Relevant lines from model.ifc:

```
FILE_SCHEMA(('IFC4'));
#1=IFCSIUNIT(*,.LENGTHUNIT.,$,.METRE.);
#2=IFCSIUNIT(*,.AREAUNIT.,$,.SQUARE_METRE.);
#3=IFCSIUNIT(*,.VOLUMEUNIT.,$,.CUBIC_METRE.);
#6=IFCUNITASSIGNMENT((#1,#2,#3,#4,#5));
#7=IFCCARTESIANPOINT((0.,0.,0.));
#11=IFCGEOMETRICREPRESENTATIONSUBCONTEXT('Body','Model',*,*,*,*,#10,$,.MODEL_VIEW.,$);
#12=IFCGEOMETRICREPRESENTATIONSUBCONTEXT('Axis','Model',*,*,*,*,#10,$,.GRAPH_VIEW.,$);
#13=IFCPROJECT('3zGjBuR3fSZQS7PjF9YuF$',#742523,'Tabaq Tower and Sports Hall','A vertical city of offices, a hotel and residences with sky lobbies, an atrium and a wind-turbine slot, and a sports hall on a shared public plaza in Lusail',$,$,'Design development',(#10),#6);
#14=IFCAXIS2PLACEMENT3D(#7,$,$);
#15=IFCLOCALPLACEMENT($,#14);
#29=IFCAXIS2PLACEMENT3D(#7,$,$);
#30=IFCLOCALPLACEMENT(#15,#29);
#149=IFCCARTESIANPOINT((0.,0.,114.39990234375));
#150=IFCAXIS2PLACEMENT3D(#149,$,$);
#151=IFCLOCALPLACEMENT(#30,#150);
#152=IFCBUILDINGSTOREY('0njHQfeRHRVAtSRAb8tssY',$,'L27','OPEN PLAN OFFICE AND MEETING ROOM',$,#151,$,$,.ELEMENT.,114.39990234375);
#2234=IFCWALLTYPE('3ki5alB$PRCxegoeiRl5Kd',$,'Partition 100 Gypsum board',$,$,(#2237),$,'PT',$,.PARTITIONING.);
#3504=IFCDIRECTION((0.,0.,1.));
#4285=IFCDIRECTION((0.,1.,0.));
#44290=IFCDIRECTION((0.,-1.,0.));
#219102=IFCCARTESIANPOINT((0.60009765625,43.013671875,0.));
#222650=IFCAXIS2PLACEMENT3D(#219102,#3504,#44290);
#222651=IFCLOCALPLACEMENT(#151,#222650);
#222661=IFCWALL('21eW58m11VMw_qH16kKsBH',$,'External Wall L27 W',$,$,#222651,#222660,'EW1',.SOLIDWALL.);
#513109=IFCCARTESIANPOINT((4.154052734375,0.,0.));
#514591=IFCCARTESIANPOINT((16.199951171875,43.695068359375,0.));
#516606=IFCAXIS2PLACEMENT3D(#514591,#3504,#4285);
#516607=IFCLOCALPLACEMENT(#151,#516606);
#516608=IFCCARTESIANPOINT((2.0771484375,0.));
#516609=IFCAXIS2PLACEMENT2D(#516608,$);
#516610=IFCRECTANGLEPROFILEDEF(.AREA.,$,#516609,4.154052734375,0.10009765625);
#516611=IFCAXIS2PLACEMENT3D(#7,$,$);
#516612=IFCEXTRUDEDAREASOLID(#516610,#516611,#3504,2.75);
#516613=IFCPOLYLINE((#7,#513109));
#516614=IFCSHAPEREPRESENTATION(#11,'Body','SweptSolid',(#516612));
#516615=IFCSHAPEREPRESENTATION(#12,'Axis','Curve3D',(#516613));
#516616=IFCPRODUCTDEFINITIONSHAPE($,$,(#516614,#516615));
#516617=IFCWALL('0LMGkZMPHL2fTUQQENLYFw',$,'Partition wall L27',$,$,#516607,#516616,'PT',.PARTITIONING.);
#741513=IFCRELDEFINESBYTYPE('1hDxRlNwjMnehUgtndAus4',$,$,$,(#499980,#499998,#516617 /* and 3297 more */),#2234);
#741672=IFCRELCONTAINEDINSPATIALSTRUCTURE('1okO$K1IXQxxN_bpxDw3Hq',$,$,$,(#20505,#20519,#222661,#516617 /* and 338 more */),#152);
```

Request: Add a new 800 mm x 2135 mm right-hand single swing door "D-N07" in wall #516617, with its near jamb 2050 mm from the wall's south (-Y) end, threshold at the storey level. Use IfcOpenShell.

```python
import numpy as np
import ifcopenshell
import ifcopenshell.api.feature
import ifcopenshell.api.geometry
import ifcopenshell.api.root
import ifcopenshell.api.spatial
import ifcopenshell.geom
import ifcopenshell.util.element
import ifcopenshell.util.placement
import ifcopenshell.util.representation
import ifcopenshell.util.shape
import ifcopenshell.util.unit

model = ifcopenshell.open("model.ifc")
unit_scale = ifcopenshell.util.unit.calculate_unit_scale(model)
settings = ifcopenshell.geom.settings()


def volume(element):
    """Net volume in cubic metres, openings subtracted."""
    shape = ifcopenshell.geom.create_shape(settings, element)
    return ifcopenshell.util.shape.get_volume(shape.geometry)


wall = model.by_id(516617)
storey = ifcopenshell.util.element.get_container(wall, ifc_class="IfcBuildingStorey")
context = ifcopenshell.util.representation.get_context(model, "Model", "Body", "MODEL_VIEW")
before = volume(wall)

width, height, from_end, sill = 0.8, 2.135, 2.05, 0.0  # metres

# The wall runs along its own X axis, and the end named is its -X end.
wall_shape = ifcopenshell.geom.create_shape(settings, wall)
x, y, z = ifcopenshell.util.shape.get_vertices(wall_shape.geometry).T
start = x.min() + from_end
face, thickness = float(y.min()), float(y.max() - y.min())
wall_matrix = ifcopenshell.util.placement.get_local_placement(wall.ObjectPlacement)
level = ifcopenshell.util.placement.get_local_placement(storey.ObjectPlacement)[2, 3]


def in_wall(x, y):
    """Placement at x, y metres in the wall's axes, at sill height."""
    matrix = wall_matrix.copy()
    matrix[:, 3] = wall_matrix @ np.array([x / unit_scale, y / unit_scale, 0.0, 1.0])
    matrix[2, 3] = level + sill / unit_scale
    return matrix


# Opening: a box that overshoots both wall faces by 50 mm.
opening = ifcopenshell.api.root.create_entity(model, ifc_class="IfcOpeningElement", predefined_type="OPENING")
box = ifcopenshell.api.geometry.add_wall_representation(
    model, context=context, length=width, height=height, thickness=thickness + 0.1
)
ifcopenshell.api.geometry.assign_representation(model, product=opening, representation=box)
ifcopenshell.api.geometry.edit_object_placement(model, product=opening, matrix=in_wall(start, face - 0.05), is_si=False)
ifcopenshell.api.feature.add_feature(model, feature=opening, element=wall)

door = ifcopenshell.api.root.create_entity(model, ifc_class="IfcDoor", name="D-N07", predefined_type="DOOR")
door.OverallWidth, door.OverallHeight = width / unit_scale, height / unit_scale
door.OperationType = "SINGLE_SWING_RIGHT"
body = ifcopenshell.api.geometry.add_door_representation(
    model,
    context=context,
    overall_width=door.OverallWidth,
    overall_height=door.OverallHeight,
    operation_type="SINGLE_SWING_RIGHT",
    lining_properties={"LiningDepth": thickness / unit_scale, "ThresholdDepth": thickness / unit_scale},
)
ifcopenshell.api.geometry.assign_representation(model, product=door, representation=body)
ifcopenshell.api.spatial.assign_container(model, products=[door], relating_structure=storey)
ifcopenshell.api.feature.add_filling(model, opening=opening, element=door)

# The lining spans the wall, so the door starts at the wall face.
ifcopenshell.api.geometry.edit_object_placement(model, product=door, matrix=in_wall(start, face), is_si=False)

after = volume(wall)

print(f"wall volume {before:.3f} -> {after:.3f} m3")

model.write("model_updated.ifc")
```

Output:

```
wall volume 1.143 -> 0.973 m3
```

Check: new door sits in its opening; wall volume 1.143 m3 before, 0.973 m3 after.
